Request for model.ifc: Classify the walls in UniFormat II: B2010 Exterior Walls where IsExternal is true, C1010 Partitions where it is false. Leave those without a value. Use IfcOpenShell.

First a look at what the model holds.

```python
import ifcopenshell
import ifcopenshell.util.element

model = ifcopenshell.open("model.ifc")
print(model.schema)
print("classifications:", [c.Name for c in model.by_type("IfcClassification")])
values = [ifcopenshell.util.element.get_pset(e, "Pset_WallCommon", "IsExternal") for e in model.by_type("IfcWall")]
for value in (True, False, None):
    print("IsExternal", value, values.count(value))
```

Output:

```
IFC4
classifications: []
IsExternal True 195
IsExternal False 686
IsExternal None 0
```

```python
import ifcopenshell
import ifcopenshell.api.classification
import ifcopenshell.util.element

model = ifcopenshell.open("model.ifc")

system = ifcopenshell.api.classification.add_classification(model, classification="UniFormat II")

walls = model.by_type("IfcWall")
external = {e: ifcopenshell.util.element.get_pset(e, "Pset_WallCommon", "IsExternal") for e in walls}
for flag, code, name in ((True, "B2010", "Exterior Walls"), (False, "C1010", "Partitions")):
    products = [e for e in walls if external[e] is flag]
    ifcopenshell.api.classification.add_reference(
        model, products=products, classification=system, identification=code, name=name
    )
    print(code, len(products))

model.write("model_edited.ifc")
```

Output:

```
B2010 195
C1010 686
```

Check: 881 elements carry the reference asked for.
